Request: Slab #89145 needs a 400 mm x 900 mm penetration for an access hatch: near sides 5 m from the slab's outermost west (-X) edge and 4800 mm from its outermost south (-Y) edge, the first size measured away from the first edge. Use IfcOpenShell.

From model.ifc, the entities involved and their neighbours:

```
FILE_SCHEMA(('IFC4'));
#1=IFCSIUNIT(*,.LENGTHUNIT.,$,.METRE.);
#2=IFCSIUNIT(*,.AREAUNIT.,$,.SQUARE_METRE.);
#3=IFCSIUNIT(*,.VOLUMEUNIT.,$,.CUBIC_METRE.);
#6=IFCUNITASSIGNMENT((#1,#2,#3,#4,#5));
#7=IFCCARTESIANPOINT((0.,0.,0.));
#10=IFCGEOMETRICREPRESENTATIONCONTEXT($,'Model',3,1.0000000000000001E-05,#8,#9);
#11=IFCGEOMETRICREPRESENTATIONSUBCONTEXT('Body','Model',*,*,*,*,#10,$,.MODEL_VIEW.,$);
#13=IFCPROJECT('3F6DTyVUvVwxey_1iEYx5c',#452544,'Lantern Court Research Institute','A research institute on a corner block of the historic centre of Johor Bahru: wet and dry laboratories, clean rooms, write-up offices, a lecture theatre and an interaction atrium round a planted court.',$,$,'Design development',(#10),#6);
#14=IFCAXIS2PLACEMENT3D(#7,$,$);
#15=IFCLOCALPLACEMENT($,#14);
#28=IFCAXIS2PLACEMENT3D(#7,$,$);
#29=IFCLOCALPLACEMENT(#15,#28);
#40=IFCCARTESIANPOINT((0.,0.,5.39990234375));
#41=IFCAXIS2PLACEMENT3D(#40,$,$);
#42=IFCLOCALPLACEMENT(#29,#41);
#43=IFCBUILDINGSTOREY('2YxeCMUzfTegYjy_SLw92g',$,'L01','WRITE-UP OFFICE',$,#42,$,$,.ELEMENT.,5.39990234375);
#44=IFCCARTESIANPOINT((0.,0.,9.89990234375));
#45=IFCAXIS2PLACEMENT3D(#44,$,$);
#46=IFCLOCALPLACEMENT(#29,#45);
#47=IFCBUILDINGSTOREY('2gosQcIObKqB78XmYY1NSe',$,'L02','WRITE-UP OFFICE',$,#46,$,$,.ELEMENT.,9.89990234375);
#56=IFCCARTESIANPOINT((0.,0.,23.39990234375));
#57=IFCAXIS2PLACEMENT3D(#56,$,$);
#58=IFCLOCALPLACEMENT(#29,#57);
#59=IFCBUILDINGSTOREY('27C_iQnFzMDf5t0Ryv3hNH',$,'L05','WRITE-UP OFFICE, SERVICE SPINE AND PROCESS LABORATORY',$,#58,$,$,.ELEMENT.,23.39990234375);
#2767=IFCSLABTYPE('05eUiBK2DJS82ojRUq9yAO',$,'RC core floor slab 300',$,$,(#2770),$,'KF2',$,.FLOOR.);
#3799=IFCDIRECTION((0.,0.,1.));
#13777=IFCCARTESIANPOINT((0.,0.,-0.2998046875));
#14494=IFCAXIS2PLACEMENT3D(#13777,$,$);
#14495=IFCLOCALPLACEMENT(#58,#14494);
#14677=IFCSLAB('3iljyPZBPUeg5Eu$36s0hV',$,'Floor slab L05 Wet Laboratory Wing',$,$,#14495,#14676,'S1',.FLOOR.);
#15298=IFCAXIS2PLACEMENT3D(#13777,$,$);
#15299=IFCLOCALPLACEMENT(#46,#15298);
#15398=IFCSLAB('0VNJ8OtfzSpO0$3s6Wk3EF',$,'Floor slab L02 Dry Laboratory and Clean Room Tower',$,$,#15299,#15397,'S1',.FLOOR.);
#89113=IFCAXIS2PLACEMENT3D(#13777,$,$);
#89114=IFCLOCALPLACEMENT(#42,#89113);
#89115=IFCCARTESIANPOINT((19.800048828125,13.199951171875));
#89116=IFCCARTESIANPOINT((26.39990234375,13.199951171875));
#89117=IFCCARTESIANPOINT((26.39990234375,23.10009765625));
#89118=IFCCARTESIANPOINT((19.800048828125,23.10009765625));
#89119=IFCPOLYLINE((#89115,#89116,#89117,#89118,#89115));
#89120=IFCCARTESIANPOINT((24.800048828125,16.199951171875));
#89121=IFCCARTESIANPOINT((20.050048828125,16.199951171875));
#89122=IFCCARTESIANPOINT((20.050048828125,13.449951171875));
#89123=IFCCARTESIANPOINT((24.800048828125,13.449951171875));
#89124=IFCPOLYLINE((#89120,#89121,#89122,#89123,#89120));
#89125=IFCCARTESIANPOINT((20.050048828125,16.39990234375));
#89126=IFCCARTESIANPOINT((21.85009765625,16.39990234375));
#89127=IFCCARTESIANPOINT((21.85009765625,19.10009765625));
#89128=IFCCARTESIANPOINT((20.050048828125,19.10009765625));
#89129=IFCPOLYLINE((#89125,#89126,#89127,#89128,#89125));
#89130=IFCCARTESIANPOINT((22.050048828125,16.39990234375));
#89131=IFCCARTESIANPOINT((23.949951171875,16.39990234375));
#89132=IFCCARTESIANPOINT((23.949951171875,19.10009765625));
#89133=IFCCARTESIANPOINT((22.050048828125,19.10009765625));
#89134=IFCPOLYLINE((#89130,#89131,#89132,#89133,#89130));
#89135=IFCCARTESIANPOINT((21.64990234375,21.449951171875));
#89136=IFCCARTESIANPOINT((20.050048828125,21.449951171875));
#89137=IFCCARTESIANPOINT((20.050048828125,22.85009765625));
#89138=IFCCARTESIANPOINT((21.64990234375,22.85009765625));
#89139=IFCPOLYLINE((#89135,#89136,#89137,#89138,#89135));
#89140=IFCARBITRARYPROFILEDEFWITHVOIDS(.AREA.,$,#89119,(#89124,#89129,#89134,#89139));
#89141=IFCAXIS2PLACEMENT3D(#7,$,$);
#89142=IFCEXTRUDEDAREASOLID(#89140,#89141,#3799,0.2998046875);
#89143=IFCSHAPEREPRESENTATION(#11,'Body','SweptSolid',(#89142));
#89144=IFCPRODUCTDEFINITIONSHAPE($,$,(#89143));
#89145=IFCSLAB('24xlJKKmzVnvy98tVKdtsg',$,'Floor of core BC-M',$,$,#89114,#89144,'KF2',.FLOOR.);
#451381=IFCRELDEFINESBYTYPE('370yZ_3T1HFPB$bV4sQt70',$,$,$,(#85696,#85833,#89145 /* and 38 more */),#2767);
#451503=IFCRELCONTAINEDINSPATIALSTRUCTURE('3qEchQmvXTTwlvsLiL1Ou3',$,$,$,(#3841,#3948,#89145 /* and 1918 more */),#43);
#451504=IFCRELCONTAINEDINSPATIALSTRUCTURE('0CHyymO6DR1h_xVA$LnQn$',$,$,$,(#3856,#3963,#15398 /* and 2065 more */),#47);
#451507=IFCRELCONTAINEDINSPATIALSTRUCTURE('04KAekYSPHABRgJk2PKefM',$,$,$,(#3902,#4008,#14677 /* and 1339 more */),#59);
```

```python
import numpy as np
import ifcopenshell
import ifcopenshell.api.feature
import ifcopenshell.api.geometry
import ifcopenshell.api.root
import ifcopenshell.geom
import ifcopenshell.util.placement
import ifcopenshell.util.representation
import ifcopenshell.util.shape
import ifcopenshell.util.unit

model = ifcopenshell.open("model.ifc")
unit_scale = ifcopenshell.util.unit.calculate_unit_scale(model)
settings = ifcopenshell.geom.settings()


def volume(element):
    """Net volume in cubic metres, openings subtracted."""
    shape = ifcopenshell.geom.create_shape(settings, element)
    return ifcopenshell.util.shape.get_volume(shape.geometry)


slab = model.by_guid("24xlJKKmzVnvy98tVKdtsg")
before = volume(slab)

# Extent in the slab's own axes, in metres. The edges named are its -X and -Y sides.
slab_shape = ifcopenshell.geom.create_shape(settings, slab)
vertices = ifcopenshell.util.shape.get_vertices(slab_shape.geometry)
x_min, y_min, bottom = vertices.min(axis=0)
top = vertices[:, 2].max()

opening = ifcopenshell.api.root.create_entity(model, ifc_class="IfcOpeningElement", name="Access hatch opening", predefined_type="OPENING")
context = ifcopenshell.util.representation.get_context(model, "Model", "Body", "MODEL_VIEW")
width, depth = 0.4, 0.9
outline = [(0.0, 0.0), (width, 0.0), (width, depth), (0.0, depth), (0.0, 0.0)]
# Overshoot both faces by 50 mm so the cut is clean.
shape = ifcopenshell.api.geometry.add_slab_representation(
    model, context=context, depth=top - bottom + 0.1, polyline=outline
)
ifcopenshell.api.geometry.assign_representation(model, product=opening, representation=shape)

matrix = ifcopenshell.util.placement.get_local_placement(slab.ObjectPlacement)
matrix[:, 3] = matrix @ np.append(np.array([x_min + 5, y_min + 4.8, bottom - 0.05]) / unit_scale, 1.0)
ifcopenshell.api.geometry.edit_object_placement(model, product=opening, matrix=matrix, is_si=False)
ifcopenshell.api.feature.add_feature(model, feature=opening, element=slab)

after = volume(slab)

print(f"slab volume {before:.3f} -> {after:.3f} m3")

model.write("model_updated.ifc")
```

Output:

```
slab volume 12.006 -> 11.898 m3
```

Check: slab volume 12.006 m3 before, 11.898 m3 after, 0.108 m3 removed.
